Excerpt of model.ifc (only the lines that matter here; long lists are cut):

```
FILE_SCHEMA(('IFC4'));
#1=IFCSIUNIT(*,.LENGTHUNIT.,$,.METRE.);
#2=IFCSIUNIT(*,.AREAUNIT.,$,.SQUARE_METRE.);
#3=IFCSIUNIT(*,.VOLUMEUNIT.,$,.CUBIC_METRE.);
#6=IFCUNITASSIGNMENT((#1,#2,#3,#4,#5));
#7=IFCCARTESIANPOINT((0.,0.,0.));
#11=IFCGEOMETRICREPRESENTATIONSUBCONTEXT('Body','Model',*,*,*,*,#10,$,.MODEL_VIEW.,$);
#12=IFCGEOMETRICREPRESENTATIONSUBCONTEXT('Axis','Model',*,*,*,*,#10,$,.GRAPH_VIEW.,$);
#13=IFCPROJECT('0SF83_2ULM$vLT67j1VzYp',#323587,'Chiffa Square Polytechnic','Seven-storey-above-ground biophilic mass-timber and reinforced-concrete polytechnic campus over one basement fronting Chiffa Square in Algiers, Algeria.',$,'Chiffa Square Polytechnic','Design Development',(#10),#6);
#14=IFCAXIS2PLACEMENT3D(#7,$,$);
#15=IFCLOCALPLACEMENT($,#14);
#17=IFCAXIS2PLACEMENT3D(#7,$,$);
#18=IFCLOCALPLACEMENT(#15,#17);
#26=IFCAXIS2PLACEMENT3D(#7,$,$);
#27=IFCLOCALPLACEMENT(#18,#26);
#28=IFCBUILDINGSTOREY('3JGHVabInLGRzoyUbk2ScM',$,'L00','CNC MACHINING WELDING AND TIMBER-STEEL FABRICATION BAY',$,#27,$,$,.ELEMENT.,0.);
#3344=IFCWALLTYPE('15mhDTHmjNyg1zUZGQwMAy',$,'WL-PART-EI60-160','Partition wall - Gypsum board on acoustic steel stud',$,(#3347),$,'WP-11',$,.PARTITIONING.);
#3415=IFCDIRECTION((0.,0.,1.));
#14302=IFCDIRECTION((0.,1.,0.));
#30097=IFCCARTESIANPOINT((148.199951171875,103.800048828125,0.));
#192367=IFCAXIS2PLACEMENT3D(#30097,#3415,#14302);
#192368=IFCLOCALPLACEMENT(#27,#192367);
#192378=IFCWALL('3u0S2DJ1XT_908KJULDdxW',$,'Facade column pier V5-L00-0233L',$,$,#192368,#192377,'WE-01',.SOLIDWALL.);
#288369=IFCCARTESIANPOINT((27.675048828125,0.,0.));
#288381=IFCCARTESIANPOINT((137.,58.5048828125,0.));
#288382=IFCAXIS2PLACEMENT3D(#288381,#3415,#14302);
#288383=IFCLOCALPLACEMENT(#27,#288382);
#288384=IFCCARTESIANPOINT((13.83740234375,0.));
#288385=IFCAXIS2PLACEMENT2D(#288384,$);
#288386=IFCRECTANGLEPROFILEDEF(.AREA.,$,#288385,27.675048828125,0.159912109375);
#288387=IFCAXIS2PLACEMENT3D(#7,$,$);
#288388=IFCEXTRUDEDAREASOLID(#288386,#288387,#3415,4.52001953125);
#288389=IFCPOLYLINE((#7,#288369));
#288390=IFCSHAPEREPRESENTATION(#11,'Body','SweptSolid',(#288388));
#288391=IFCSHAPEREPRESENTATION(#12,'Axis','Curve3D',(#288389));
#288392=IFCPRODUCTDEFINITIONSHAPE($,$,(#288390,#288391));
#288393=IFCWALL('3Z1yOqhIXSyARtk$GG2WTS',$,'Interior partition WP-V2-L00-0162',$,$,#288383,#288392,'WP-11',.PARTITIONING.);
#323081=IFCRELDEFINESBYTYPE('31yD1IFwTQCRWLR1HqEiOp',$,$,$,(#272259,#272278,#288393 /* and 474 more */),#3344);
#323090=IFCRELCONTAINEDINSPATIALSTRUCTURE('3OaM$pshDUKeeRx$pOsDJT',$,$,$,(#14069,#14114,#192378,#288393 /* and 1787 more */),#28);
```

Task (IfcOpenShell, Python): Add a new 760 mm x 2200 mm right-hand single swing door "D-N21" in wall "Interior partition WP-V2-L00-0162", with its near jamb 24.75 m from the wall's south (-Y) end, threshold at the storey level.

```python
import numpy as np
import ifcopenshell
import ifcopenshell.api.feature
import ifcopenshell.api.geometry
import ifcopenshell.api.root
import ifcopenshell.api.spatial
import ifcopenshell.geom
import ifcopenshell.util.element
import ifcopenshell.util.placement
import ifcopenshell.util.representation
import ifcopenshell.util.shape
import ifcopenshell.util.unit

model = ifcopenshell.open("model.ifc")
unit_scale = ifcopenshell.util.unit.calculate_unit_scale(model)
settings = ifcopenshell.geom.settings()


def volume(element):
    """Net volume in cubic metres, openings subtracted."""
    shape = ifcopenshell.geom.create_shape(settings, element)
    return ifcopenshell.util.shape.get_volume(shape.geometry)


wall = model.by_guid("3Z1yOqhIXSyARtk$GG2WTS")
storey = ifcopenshell.util.element.get_container(wall, ifc_class="IfcBuildingStorey")
context = ifcopenshell.util.representation.get_context(model, "Model", "Body", "MODEL_VIEW")
before = volume(wall)

width, height, from_end, sill = 0.76, 2.2, 24.75, 0.0  # metres

# The wall runs along its own X axis, and the end named is its -X end.
wall_shape = ifcopenshell.geom.create_shape(settings, wall)
x, y, z = ifcopenshell.util.shape.get_vertices(wall_shape.geometry).T
start = x.min() + from_end
face, thickness = float(y.min()), float(y.max() - y.min())
wall_matrix = ifcopenshell.util.placement.get_local_placement(wall.ObjectPlacement)
level = ifcopenshell.util.placement.get_local_placement(storey.ObjectPlacement)[2, 3]


def in_wall(x, y):
    """Placement at x, y metres in the wall's axes, at sill height."""
    matrix = wall_matrix.copy()
    matrix[:, 3] = wall_matrix @ np.array([x / unit_scale, y / unit_scale, 0.0, 1.0])
    matrix[2, 3] = level + sill / unit_scale
    return matrix


# Opening: a box that overshoots both wall faces by 50 mm.
opening = ifcopenshell.api.root.create_entity(model, ifc_class="IfcOpeningElement", predefined_type="OPENING")
box = ifcopenshell.api.geometry.add_wall_representation(
    model, context=context, length=width, height=height, thickness=thickness + 0.1
)
ifcopenshell.api.geometry.assign_representation(model, product=opening, representation=box)
ifcopenshell.api.geometry.edit_object_placement(model, product=opening, matrix=in_wall(start, face - 0.05), is_si=False)
ifcopenshell.api.feature.add_feature(model, feature=opening, element=wall)

door = ifcopenshell.api.root.create_entity(model, ifc_class="IfcDoor", name="D-N21", predefined_type="DOOR")
door.OverallWidth, door.OverallHeight = width / unit_scale, height / unit_scale
door.OperationType = "SINGLE_SWING_RIGHT"
body = ifcopenshell.api.geometry.add_door_representation(
    model,
    context=context,
    overall_width=door.OverallWidth,
    overall_height=door.OverallHeight,
    operation_type="SINGLE_SWING_RIGHT",
    lining_properties={"LiningDepth": thickness / unit_scale, "ThresholdDepth": thickness / unit_scale},
)
ifcopenshell.api.geometry.assign_representation(model, product=door, representation=body)
ifcopenshell.api.spatial.assign_container(model, products=[door], relating_structure=storey)
ifcopenshell.api.feature.add_filling(model, opening=opening, element=door)

# The lining spans the wall, so the door starts at the wall face.
ifcopenshell.api.geometry.edit_object_placement(model, product=door, matrix=in_wall(start, face), is_si=False)

after = volume(wall)

print(f"wall volume {before:.3f} -> {after:.3f} m3")

model.write("model-out.ifc")
```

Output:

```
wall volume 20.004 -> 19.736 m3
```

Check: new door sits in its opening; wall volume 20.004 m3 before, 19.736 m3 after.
